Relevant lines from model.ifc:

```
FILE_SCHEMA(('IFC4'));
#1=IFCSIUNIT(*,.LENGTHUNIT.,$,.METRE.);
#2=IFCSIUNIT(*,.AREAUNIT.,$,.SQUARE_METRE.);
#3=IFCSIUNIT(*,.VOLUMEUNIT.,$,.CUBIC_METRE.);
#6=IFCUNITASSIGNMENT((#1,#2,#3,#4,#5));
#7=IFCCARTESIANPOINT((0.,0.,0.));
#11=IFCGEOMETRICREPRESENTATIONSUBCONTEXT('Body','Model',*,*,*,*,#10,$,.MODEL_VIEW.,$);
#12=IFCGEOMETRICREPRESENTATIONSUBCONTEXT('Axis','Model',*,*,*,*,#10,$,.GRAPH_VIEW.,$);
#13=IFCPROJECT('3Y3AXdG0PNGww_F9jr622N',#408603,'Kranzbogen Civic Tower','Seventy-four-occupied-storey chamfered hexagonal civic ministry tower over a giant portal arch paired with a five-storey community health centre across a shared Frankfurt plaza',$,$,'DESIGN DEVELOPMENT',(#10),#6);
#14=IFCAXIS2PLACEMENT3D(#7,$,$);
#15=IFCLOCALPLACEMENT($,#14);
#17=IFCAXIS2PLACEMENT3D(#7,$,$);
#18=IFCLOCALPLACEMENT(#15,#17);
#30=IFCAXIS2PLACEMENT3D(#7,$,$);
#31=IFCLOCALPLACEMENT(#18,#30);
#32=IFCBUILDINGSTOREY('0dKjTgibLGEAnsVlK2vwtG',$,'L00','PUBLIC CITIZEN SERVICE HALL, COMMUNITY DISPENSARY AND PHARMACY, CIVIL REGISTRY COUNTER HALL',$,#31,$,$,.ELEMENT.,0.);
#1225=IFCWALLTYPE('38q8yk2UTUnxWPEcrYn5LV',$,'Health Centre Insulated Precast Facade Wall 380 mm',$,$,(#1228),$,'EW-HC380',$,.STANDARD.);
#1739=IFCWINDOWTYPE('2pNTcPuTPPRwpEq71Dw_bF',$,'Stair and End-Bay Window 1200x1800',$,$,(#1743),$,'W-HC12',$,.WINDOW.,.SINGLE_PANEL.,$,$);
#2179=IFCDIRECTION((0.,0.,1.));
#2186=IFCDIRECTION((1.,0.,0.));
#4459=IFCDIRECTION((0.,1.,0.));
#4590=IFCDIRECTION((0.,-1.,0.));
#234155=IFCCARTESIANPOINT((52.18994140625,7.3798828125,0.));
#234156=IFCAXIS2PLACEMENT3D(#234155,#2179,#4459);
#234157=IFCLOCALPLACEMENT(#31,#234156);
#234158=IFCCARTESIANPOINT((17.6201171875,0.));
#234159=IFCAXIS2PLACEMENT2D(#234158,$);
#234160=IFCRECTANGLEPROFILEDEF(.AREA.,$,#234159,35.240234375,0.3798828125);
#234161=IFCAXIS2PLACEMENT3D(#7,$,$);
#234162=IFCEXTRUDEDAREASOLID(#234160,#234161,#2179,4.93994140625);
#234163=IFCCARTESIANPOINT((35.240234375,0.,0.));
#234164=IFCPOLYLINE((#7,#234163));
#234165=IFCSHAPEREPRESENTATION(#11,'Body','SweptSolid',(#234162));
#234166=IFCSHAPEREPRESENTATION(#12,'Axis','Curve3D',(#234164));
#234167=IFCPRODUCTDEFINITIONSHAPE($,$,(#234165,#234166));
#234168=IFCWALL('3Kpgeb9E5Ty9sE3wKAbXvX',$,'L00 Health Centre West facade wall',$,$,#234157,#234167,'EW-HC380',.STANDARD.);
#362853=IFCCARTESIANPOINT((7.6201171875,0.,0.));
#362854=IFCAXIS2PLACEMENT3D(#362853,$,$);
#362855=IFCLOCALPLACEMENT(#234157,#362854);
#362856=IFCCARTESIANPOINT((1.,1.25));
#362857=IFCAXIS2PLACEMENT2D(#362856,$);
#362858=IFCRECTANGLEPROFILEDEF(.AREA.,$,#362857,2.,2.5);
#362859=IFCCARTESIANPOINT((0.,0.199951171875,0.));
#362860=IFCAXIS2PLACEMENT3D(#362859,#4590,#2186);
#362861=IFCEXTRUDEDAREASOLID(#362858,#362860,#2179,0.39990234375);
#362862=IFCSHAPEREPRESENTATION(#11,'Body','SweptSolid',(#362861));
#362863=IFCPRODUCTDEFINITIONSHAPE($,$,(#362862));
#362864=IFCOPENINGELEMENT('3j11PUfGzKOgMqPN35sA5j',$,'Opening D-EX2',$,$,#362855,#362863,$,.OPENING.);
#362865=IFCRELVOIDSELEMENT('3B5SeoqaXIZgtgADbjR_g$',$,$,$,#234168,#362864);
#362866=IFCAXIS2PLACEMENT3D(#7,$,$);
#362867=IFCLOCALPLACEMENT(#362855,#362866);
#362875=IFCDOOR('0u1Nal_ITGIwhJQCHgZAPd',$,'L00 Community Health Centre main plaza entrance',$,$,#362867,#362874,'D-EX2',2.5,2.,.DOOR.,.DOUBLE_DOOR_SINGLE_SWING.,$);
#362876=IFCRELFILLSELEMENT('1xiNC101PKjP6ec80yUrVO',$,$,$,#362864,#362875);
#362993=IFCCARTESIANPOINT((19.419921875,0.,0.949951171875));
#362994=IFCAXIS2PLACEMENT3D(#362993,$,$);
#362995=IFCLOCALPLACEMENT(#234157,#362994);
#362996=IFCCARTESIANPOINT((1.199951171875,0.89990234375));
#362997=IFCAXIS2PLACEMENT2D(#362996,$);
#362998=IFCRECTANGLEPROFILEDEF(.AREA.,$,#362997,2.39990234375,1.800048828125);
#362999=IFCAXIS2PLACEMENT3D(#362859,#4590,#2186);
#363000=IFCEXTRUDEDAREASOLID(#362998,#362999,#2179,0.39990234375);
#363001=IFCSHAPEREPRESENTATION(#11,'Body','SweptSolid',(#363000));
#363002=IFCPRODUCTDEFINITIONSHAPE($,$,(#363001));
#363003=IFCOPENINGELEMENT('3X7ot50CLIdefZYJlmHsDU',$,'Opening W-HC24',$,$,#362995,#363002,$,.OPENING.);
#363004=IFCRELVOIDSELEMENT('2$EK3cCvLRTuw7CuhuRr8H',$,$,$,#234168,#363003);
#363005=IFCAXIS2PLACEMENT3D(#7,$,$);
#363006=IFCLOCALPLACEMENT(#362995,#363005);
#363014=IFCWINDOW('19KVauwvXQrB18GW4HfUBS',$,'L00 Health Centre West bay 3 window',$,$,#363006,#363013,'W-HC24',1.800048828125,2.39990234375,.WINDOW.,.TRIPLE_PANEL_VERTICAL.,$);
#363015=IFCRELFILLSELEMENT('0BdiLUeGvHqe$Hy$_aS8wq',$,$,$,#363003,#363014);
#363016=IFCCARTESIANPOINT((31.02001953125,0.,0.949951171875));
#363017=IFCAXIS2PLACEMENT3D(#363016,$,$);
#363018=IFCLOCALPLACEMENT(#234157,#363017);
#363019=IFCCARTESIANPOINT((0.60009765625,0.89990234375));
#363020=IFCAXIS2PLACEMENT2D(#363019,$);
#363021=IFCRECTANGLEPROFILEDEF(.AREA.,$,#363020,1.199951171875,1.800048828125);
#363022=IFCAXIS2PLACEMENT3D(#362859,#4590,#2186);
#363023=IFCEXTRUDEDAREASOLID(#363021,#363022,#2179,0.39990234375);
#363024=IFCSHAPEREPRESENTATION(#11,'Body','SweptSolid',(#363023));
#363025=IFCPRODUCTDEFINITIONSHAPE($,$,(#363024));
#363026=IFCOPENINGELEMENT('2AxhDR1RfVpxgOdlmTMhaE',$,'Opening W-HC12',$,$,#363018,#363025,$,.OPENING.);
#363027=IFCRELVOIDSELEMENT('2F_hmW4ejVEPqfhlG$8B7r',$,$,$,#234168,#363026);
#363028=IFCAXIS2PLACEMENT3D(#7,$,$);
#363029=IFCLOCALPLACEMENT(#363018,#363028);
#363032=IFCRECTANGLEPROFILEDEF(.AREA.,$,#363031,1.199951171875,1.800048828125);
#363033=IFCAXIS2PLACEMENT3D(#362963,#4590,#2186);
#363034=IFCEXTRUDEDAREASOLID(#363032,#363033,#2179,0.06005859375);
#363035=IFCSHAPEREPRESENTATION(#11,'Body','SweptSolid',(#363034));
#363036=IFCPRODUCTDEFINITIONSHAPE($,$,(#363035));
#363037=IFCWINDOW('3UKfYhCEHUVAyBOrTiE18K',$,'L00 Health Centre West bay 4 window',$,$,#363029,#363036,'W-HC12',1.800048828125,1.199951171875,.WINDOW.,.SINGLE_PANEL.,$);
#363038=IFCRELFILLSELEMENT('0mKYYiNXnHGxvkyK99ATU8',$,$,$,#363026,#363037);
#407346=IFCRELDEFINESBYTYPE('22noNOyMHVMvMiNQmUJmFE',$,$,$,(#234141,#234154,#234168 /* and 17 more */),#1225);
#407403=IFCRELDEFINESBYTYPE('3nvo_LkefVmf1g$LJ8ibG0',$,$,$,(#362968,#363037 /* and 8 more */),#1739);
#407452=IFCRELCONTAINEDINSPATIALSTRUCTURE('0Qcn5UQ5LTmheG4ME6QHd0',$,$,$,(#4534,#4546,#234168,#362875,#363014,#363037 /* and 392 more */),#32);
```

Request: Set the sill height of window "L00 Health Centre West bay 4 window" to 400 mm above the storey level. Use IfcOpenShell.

```python
import numpy as np
import ifcopenshell
import ifcopenshell.api.geometry
import ifcopenshell.geom
import ifcopenshell.util.element
import ifcopenshell.util.placement
import ifcopenshell.util.shape
import ifcopenshell.util.unit

model = ifcopenshell.open("model.ifc")
unit_scale = ifcopenshell.util.unit.calculate_unit_scale(model)

window = model.by_guid("3UKfYhCEHUVAyBOrTiE18K")
opening = window.FillsVoids[0].RelatingOpeningElement
storey = ifcopenshell.util.element.get_container(window, ifc_class="IfcBuildingStorey")
level = ifcopenshell.util.placement.get_local_placement(storey.ObjectPlacement)[2, 3]

# The opening's origin need not be at the sill, so measure its lowest point.
shape = ifcopenshell.geom.create_shape(ifcopenshell.geom.settings(), opening)
bottom = ifcopenshell.util.shape.get_shape_bottom_elevation(shape, shape.geometry) / unit_scale
dz = level + 0.4 - bottom

shift = np.array([0.0, 0.0, dz])
# The window is placed relative to its opening, so it follows when the opening moves.
matrix = ifcopenshell.util.placement.get_local_placement(opening.ObjectPlacement)
matrix[:3, 3] += shift
ifcopenshell.api.geometry.edit_object_placement(
    model, product=opening, matrix=matrix, is_si=False, should_transform_children=True
)

print(f"moved by {dz * unit_scale:+.3f} m")

model.write("model_v2.ifc")
```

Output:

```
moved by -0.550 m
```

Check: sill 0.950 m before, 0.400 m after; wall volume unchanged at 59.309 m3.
